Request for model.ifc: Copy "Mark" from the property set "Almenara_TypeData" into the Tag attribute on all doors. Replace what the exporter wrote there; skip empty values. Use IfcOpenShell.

First a look at what the model holds.

```python
import ifcopenshell
import ifcopenshell.util.element

model = ifcopenshell.open("model.ifc")
print(model.schema)
doors = model.by_type("IfcDoor")
print(len(doors), "doors")
for e in doors[:8]:
    source = ifcopenshell.util.element.get_pset(e, "Almenara_TypeData", "Mark")
    target = e.Tag
    print(e.id(), repr(source), repr(target), sep=" | ")
```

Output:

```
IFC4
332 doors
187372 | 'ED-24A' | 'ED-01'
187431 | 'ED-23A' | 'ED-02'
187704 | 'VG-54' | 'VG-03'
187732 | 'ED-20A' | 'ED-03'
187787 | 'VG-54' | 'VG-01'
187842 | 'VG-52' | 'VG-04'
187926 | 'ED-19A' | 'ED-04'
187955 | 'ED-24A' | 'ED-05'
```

```python
import ifcopenshell
import ifcopenshell.util.element

model = ifcopenshell.open("model.ifc")

count = 0
for e in model.by_type("IfcDoor"):
    value = ifcopenshell.util.element.get_pset(e, "Almenara_TypeData", "Mark")
    current = e.Tag
    if not value or not value.strip() or current == value:
        continue
    e.Tag = value
    count += 1

print(count, "doors updated")

model.write("model_edited.ifc")
```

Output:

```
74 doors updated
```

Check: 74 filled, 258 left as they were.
